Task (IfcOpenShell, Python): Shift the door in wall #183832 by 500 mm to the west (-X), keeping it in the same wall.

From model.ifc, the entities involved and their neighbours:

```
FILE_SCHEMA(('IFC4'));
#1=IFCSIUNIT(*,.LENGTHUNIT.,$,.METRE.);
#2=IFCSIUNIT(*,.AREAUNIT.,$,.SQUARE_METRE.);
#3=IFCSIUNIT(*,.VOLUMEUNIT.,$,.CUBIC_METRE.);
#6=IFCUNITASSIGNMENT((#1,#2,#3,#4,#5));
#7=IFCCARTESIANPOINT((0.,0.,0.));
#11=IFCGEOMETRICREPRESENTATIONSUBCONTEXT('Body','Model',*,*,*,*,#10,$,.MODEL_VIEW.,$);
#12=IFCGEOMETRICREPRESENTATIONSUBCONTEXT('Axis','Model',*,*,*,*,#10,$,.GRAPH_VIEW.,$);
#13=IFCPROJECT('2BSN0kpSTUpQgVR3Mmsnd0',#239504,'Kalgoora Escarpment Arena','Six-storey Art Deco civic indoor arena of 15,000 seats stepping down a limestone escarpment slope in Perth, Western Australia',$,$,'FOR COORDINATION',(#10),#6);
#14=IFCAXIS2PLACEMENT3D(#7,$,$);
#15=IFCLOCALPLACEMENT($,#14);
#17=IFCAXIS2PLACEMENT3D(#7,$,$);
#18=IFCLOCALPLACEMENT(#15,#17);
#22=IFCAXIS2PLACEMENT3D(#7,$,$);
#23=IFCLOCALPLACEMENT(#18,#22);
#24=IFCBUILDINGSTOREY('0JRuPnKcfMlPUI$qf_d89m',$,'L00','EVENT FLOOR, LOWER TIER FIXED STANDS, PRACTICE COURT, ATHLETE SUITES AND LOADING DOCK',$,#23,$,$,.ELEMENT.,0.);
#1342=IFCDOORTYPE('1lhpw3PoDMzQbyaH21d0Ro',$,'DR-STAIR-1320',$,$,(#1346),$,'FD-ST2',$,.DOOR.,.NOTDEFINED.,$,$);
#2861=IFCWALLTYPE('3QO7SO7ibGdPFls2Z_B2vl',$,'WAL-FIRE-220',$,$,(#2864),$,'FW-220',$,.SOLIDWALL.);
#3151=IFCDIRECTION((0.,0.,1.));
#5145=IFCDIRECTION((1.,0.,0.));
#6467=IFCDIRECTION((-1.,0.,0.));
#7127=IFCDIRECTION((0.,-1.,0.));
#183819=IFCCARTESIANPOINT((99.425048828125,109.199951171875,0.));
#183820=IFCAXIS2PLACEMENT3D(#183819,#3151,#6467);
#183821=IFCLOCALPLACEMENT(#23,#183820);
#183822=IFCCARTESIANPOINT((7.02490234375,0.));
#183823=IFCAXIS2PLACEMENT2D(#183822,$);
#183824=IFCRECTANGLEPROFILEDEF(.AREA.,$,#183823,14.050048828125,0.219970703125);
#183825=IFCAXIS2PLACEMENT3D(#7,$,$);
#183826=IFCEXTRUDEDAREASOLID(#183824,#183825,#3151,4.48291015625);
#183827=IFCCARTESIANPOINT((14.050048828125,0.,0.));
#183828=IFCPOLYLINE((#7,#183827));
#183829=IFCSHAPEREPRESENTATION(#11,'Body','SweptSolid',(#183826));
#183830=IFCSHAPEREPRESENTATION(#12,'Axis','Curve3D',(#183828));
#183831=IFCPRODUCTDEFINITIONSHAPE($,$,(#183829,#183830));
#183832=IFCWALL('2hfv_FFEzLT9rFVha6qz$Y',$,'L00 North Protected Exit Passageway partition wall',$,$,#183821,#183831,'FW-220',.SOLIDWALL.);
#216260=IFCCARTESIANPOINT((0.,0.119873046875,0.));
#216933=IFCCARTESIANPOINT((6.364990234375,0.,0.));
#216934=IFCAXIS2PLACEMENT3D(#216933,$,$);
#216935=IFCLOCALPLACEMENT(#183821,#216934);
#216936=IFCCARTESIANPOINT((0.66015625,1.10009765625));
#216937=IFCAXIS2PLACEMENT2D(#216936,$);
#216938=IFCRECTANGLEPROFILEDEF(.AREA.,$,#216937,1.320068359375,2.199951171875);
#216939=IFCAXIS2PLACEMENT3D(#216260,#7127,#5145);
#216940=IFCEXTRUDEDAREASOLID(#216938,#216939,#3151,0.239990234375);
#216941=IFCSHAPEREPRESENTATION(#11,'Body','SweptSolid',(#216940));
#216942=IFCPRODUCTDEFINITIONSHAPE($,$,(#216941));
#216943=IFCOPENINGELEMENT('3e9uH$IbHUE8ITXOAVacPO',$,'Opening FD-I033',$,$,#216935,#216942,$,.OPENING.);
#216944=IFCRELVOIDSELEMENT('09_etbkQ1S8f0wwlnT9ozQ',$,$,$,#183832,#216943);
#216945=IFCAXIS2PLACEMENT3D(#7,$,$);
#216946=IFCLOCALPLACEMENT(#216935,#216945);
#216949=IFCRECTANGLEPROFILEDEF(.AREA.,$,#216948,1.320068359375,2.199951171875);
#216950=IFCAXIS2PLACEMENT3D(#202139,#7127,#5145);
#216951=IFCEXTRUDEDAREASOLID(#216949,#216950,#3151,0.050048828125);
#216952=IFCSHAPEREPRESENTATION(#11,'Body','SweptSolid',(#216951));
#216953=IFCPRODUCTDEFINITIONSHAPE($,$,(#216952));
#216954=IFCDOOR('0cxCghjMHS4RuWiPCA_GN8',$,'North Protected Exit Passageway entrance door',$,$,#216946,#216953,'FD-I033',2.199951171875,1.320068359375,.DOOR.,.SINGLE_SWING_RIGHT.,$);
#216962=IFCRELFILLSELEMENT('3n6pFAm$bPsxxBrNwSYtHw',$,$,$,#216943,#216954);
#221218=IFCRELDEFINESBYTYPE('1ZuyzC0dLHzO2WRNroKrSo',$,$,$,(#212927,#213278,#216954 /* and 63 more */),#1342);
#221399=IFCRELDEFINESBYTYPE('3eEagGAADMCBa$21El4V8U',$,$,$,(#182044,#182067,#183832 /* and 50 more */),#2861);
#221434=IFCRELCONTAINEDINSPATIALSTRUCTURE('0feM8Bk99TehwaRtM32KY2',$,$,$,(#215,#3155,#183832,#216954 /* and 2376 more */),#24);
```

```python
import ifcopenshell
import ifcopenshell.api.geometry
import ifcopenshell.util.placement
import ifcopenshell.util.unit

model = ifcopenshell.open("model.ifc")
unit_scale = ifcopenshell.util.unit.calculate_unit_scale(model)

door = model.by_guid("0cxCghjMHS4RuWiPCA_GN8")
opening = door.FillsVoids[0].RelatingOpeningElement
wall = opening.VoidsElements[0].RelatingBuildingElement

wall_matrix = ifcopenshell.util.placement.get_local_placement(wall.ObjectPlacement)
shift = wall_matrix[:3, 0] * 0.5 / unit_scale
before = ifcopenshell.util.placement.get_local_placement(door.ObjectPlacement)[:3, 3].copy()

# The door is placed relative to its opening, so it follows when the opening moves.
matrix = ifcopenshell.util.placement.get_local_placement(opening.ObjectPlacement)
matrix[:3, 3] += shift
ifcopenshell.api.geometry.edit_object_placement(
    model, product=opening, matrix=matrix, is_si=False, should_transform_children=True
)

after = ifcopenshell.util.placement.get_local_placement(door.ObjectPlacement)[:3, 3]
print("door moved by", (after - before).round(3) + 0.0)

model.write("model_updated.ifc")
```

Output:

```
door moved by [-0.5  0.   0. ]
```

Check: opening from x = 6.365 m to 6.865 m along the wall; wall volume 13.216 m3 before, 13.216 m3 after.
